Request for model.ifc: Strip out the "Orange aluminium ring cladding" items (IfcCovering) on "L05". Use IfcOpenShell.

First a look at what the model holds.

```python
import ifcopenshell
import ifcopenshell.util.element

model = ifcopenshell.open("model.ifc")
print(model.schema)
storey = next(s for s in model.by_type("IfcBuildingStorey") if s.Name == "L05")
coverings = [e for e in ifcopenshell.util.element.get_decomposition(storey) if e.is_a("IfcCovering")]
seen = {}
for e in coverings:
    element_type = ifcopenshell.util.element.get_type(e)
    name = element_type.Name if element_type not in (None, e) else None
    seen[name] = seen.get(name, 0) + 1
for name, count in sorted(seen.items(), key=str):
    print(count, "x", name)
```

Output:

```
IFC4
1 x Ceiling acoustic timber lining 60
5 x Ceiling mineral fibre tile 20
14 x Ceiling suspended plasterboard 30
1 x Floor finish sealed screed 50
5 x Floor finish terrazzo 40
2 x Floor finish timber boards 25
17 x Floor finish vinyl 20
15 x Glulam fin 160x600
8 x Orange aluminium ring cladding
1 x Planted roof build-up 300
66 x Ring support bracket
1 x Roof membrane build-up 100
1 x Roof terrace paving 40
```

```python
import ifcopenshell
import ifcopenshell.api.root
import ifcopenshell.util.element

model = ifcopenshell.open("model.ifc")

storey = next(s for s in model.by_type("IfcBuildingStorey") if s.Name == "L05")
coverings = [e for e in ifcopenshell.util.element.get_decomposition(storey) if e.is_a("IfcCovering")]
targets = [e for e in coverings if (t := ifcopenshell.util.element.get_type(e)) not in (None, e) and t.Name == "Orange aluminium ring cladding"]

for e in targets:
    ifcopenshell.api.root.remove_product(model, product=e)
print(len(targets), "removed")

model.write("model_v2.ifc")
```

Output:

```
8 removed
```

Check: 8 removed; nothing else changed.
